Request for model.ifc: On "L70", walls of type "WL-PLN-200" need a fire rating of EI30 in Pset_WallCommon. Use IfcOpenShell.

First a look at what the model holds.

```python
import ifcopenshell
import ifcopenshell.util.element

model = ifcopenshell.open("model.ifc")
print(model.schema)
storey = next(s for s in model.by_type("IfcBuildingStorey") if s.Name == "L70")
walls = [e for e in ifcopenshell.util.element.get_decomposition(storey) if e.is_a("IfcWall")]
seen = {}
for e in walls:
    element_type = ifcopenshell.util.element.get_type(e)
    key = (element_type.Name if element_type != e and element_type else None, ifcopenshell.util.element.get_pset(e, "Pset_WallCommon", "FireRating"))
    seen[key] = seen.get(key, 0) + 1
for (name, value), count in sorted(seen.items(), key=str):
    print(count, "x", name, "|", value)
```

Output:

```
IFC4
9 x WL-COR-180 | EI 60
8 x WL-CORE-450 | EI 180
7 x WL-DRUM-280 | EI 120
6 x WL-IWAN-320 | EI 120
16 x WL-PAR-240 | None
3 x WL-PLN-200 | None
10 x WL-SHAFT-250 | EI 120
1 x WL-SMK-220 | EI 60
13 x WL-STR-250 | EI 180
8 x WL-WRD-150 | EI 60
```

```python
import ifcopenshell
import ifcopenshell.api.pset
import ifcopenshell.util.element

model = ifcopenshell.open("model.ifc")

storey = next(s for s in model.by_type("IfcBuildingStorey") if s.Name == "L70")
walls = [e for e in ifcopenshell.util.element.get_decomposition(storey) if e.is_a("IfcWall")]

count = 0
for e in walls:
    element_type = ifcopenshell.util.element.get_type(e)
    if element_type in (None, e) or element_type.Name != "WL-PLN-200":
        continue
    found = ifcopenshell.util.element.get_pset(e, "Pset_WallCommon", should_inherit=False)
    if found:
        pset = model.by_id(found["id"])
        if len(ifcopenshell.util.element.get_elements_by_pset(pset)) > 1:
            pset = ifcopenshell.api.pset.unshare_pset(model, products=[e], pset=pset)[0]
    else:
        pset = ifcopenshell.api.pset.add_pset(model, product=e, name="Pset_WallCommon")
    ifcopenshell.api.pset.edit_pset(model, pset=pset, properties={"FireRating": "EI30"})
    count += 1

print(count, "walls updated")

model.write("model_edited.ifc")
```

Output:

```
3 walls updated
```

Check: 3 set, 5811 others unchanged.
